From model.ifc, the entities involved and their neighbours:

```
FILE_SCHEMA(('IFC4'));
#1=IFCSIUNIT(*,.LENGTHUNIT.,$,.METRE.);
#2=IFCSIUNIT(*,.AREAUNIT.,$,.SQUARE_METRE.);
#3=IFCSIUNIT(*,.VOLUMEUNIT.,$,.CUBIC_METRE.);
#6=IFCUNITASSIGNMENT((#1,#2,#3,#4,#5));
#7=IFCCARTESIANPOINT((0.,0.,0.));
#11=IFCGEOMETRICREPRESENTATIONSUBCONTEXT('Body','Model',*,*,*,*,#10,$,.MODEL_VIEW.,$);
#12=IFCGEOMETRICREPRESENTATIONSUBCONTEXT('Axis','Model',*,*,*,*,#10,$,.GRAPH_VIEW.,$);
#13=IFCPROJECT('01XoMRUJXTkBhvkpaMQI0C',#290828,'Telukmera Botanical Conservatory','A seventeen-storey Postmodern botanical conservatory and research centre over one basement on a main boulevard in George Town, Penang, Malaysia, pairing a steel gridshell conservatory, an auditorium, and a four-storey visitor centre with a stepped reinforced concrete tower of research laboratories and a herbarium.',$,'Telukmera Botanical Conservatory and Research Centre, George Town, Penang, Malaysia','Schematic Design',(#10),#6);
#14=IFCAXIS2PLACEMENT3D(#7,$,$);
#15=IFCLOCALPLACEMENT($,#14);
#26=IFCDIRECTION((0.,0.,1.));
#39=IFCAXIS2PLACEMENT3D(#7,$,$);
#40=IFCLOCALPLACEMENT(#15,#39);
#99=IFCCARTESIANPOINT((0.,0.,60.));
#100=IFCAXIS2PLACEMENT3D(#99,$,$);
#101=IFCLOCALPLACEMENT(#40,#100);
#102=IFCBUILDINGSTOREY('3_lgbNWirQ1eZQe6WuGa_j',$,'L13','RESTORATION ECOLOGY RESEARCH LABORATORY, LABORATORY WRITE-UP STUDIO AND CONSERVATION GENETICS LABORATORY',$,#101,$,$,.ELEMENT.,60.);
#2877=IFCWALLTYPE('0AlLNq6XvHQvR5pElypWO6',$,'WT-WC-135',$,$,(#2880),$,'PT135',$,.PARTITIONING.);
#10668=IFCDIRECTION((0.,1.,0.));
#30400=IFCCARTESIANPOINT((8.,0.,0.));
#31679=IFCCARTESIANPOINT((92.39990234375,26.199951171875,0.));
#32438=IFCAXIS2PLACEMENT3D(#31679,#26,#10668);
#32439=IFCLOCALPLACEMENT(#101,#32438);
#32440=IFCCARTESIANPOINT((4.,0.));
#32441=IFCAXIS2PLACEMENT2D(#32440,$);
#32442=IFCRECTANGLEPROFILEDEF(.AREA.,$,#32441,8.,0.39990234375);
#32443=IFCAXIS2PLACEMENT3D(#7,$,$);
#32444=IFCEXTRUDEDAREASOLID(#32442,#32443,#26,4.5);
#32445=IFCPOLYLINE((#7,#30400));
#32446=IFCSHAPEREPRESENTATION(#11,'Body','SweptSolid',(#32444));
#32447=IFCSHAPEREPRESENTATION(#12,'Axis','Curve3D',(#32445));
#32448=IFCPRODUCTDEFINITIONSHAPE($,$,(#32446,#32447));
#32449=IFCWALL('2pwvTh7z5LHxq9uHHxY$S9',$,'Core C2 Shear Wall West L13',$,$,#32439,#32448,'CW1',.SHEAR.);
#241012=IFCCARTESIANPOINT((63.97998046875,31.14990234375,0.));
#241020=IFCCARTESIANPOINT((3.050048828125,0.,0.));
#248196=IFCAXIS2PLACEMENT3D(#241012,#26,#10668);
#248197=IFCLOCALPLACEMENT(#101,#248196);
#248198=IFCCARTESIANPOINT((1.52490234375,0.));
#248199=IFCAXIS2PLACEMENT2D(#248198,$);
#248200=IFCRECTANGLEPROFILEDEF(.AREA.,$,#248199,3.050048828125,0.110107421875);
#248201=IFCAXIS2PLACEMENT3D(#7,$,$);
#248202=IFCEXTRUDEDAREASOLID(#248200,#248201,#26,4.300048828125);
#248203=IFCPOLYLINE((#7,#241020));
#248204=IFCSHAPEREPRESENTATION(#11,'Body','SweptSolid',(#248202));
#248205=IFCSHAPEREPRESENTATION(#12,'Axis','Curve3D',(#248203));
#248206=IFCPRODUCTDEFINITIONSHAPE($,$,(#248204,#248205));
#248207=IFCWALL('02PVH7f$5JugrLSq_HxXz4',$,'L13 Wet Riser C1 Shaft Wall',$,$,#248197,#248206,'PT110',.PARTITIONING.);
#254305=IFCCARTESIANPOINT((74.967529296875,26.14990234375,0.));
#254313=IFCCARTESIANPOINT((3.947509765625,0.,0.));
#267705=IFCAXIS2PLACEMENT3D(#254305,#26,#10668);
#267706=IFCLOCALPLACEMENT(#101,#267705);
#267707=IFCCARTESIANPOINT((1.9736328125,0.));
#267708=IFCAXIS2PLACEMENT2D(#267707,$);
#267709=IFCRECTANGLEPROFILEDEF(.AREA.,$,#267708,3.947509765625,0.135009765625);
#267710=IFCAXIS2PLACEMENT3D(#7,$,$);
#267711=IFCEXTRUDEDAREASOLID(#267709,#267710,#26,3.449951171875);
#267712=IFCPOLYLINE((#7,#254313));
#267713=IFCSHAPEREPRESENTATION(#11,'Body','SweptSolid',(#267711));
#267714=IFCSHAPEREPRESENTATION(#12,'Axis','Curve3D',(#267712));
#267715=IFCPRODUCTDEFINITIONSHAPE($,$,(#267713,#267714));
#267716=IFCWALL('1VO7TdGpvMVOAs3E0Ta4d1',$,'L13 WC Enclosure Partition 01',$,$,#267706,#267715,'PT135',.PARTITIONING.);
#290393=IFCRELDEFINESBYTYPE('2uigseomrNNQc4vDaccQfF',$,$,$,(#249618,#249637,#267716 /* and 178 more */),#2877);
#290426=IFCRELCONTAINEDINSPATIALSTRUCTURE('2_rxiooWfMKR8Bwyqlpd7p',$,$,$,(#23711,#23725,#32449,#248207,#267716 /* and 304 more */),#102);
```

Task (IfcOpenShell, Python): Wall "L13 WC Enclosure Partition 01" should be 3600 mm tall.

```python
import ifcopenshell
import ifcopenshell.geom
import ifcopenshell.util.representation
import ifcopenshell.util.shape
import ifcopenshell.util.unit

model = ifcopenshell.open("model.ifc")
unit_scale = ifcopenshell.util.unit.calculate_unit_scale(model)
settings = ifcopenshell.geom.settings()


def volume(element):
    """Net volume in cubic metres, openings subtracted."""
    shape = ifcopenshell.geom.create_shape(settings, element)
    return ifcopenshell.util.shape.get_volume(shape.geometry)


wall = model.by_guid("1VO7TdGpvMVOAs3E0Ta4d1")
before = volume(wall)

body = ifcopenshell.util.representation.get_representation(wall, "Model", "Body")
solid = body.Items[0]
old_height = solid.Depth
solid.Depth = 3.6 / unit_scale
after = volume(wall)

print(f"height {old_height:g} -> {solid.Depth:g}, volume {before:.3f} -> {after:.3f} m3")

model.write("model_v2.ifc")
```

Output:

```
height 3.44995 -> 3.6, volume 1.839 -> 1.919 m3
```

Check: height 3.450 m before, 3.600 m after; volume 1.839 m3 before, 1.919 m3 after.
